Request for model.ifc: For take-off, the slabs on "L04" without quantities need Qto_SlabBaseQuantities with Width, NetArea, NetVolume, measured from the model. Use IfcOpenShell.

First a look at what the model holds.

```python
import ifcopenshell
import ifcopenshell.util.element
import ifcopenshell.util.unit

model = ifcopenshell.open("model.ifc")
print(model.schema)
for unit_type in ("LENGTHUNIT", "AREAUNIT", "VOLUMEUNIT"):
    print(unit_type, ifcopenshell.util.unit.calculate_unit_scale(model, unit_type))
storey = next(s for s in model.by_type("IfcBuildingStorey") if s.Name == "L04")
slabs = [e for e in ifcopenshell.util.element.get_decomposition(storey) if e.is_a("IfcSlab")]
for e in sorted(slabs, key=lambda e: e.id()):
    print(e.id(), e.is_a(), e.Name, list(ifcopenshell.util.element.get_psets(e, qtos_only=True)), sep=" | ")
```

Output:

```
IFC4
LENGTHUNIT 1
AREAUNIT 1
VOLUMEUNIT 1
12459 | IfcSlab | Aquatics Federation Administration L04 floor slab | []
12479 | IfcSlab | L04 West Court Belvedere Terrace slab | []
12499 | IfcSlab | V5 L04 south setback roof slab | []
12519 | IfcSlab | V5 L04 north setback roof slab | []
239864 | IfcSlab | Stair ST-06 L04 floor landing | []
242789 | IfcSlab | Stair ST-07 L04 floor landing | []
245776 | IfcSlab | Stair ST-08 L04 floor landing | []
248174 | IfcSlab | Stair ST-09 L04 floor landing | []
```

```python
import ifcopenshell
import ifcopenshell.api.pset
import ifcopenshell.geom
import ifcopenshell.util.element
import ifcopenshell.util.shape
import ifcopenshell.util.unit

model = ifcopenshell.open("model.ifc")
unit_scale = ifcopenshell.util.unit.calculate_unit_scale(model)
area_scale = ifcopenshell.util.unit.calculate_unit_scale(model, "AREAUNIT")
volume_scale = ifcopenshell.util.unit.calculate_unit_scale(model, "VOLUMEUNIT")
settings = ifcopenshell.geom.settings()

storey = next(s for s in model.by_type("IfcBuildingStorey") if s.Name == "L04")
slabs = [e for e in ifcopenshell.util.element.get_decomposition(storey) if e.is_a("IfcSlab")]

for e in sorted(slabs, key=lambda e: e.id()):
    if ifcopenshell.util.element.get_psets(e, qtos_only=True, should_inherit=False):
        continue
    # Geometry comes back in metres, in the element's own axes.
    shape = ifcopenshell.geom.create_shape(settings, e)
    values = {
        "Width": ifcopenshell.util.shape.get_z(shape.geometry) / unit_scale,
        "NetArea": ifcopenshell.util.shape.get_footprint_area(shape.geometry) / area_scale,
        "NetVolume": ifcopenshell.util.shape.get_volume(shape.geometry) / volume_scale,
    }
    qto = ifcopenshell.api.pset.add_qto(model, product=e, name="Qto_SlabBaseQuantities")
    ifcopenshell.api.pset.edit_qto(model, qto=qto, properties=values)
    print(e.id(), {k: round(v, 3) for k, v in values.items()})

model.write("model_v2.ifc")
```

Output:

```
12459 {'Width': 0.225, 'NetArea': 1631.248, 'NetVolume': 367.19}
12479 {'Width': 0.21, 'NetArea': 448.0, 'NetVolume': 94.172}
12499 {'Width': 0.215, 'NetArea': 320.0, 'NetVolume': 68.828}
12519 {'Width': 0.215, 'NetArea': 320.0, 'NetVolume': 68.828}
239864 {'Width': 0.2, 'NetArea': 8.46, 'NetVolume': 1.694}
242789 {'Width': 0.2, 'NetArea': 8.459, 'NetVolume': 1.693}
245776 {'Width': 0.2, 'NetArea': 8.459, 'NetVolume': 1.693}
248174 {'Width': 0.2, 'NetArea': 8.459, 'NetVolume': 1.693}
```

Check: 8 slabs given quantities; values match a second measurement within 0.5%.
